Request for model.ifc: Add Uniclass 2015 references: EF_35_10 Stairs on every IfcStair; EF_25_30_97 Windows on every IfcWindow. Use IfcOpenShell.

First a look at what the model holds.

```python
import ifcopenshell

model = ifcopenshell.open("model.ifc")
print(model.schema)
print("classifications:", [c.Name for c in model.by_type("IfcClassification")])
for ifc_class in ("IfcDoor", "IfcRoof", "IfcStair", "IfcWall", "IfcWindow"):
    print(ifc_class, len(model.by_type(ifc_class)))
```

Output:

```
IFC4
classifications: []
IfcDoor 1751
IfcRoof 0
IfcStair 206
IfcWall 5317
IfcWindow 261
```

```python
import ifcopenshell
import ifcopenshell.api.classification

model = ifcopenshell.open("model.ifc")

system = ifcopenshell.api.classification.add_classification(model, classification="Uniclass 2015")

codes = {
    "IfcStair": ("EF_35_10", "Stairs"),
    "IfcWindow": ("EF_25_30_97", "Windows"),
}
for ifc_class, (code, name) in codes.items():
    products = model.by_type(ifc_class)
    ifcopenshell.api.classification.add_reference(
        model, products=products, classification=system, identification=code, name=name
    )
    print(code, len(products))

model.write("model_rev.ifc")
```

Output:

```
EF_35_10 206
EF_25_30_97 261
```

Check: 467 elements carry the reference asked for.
